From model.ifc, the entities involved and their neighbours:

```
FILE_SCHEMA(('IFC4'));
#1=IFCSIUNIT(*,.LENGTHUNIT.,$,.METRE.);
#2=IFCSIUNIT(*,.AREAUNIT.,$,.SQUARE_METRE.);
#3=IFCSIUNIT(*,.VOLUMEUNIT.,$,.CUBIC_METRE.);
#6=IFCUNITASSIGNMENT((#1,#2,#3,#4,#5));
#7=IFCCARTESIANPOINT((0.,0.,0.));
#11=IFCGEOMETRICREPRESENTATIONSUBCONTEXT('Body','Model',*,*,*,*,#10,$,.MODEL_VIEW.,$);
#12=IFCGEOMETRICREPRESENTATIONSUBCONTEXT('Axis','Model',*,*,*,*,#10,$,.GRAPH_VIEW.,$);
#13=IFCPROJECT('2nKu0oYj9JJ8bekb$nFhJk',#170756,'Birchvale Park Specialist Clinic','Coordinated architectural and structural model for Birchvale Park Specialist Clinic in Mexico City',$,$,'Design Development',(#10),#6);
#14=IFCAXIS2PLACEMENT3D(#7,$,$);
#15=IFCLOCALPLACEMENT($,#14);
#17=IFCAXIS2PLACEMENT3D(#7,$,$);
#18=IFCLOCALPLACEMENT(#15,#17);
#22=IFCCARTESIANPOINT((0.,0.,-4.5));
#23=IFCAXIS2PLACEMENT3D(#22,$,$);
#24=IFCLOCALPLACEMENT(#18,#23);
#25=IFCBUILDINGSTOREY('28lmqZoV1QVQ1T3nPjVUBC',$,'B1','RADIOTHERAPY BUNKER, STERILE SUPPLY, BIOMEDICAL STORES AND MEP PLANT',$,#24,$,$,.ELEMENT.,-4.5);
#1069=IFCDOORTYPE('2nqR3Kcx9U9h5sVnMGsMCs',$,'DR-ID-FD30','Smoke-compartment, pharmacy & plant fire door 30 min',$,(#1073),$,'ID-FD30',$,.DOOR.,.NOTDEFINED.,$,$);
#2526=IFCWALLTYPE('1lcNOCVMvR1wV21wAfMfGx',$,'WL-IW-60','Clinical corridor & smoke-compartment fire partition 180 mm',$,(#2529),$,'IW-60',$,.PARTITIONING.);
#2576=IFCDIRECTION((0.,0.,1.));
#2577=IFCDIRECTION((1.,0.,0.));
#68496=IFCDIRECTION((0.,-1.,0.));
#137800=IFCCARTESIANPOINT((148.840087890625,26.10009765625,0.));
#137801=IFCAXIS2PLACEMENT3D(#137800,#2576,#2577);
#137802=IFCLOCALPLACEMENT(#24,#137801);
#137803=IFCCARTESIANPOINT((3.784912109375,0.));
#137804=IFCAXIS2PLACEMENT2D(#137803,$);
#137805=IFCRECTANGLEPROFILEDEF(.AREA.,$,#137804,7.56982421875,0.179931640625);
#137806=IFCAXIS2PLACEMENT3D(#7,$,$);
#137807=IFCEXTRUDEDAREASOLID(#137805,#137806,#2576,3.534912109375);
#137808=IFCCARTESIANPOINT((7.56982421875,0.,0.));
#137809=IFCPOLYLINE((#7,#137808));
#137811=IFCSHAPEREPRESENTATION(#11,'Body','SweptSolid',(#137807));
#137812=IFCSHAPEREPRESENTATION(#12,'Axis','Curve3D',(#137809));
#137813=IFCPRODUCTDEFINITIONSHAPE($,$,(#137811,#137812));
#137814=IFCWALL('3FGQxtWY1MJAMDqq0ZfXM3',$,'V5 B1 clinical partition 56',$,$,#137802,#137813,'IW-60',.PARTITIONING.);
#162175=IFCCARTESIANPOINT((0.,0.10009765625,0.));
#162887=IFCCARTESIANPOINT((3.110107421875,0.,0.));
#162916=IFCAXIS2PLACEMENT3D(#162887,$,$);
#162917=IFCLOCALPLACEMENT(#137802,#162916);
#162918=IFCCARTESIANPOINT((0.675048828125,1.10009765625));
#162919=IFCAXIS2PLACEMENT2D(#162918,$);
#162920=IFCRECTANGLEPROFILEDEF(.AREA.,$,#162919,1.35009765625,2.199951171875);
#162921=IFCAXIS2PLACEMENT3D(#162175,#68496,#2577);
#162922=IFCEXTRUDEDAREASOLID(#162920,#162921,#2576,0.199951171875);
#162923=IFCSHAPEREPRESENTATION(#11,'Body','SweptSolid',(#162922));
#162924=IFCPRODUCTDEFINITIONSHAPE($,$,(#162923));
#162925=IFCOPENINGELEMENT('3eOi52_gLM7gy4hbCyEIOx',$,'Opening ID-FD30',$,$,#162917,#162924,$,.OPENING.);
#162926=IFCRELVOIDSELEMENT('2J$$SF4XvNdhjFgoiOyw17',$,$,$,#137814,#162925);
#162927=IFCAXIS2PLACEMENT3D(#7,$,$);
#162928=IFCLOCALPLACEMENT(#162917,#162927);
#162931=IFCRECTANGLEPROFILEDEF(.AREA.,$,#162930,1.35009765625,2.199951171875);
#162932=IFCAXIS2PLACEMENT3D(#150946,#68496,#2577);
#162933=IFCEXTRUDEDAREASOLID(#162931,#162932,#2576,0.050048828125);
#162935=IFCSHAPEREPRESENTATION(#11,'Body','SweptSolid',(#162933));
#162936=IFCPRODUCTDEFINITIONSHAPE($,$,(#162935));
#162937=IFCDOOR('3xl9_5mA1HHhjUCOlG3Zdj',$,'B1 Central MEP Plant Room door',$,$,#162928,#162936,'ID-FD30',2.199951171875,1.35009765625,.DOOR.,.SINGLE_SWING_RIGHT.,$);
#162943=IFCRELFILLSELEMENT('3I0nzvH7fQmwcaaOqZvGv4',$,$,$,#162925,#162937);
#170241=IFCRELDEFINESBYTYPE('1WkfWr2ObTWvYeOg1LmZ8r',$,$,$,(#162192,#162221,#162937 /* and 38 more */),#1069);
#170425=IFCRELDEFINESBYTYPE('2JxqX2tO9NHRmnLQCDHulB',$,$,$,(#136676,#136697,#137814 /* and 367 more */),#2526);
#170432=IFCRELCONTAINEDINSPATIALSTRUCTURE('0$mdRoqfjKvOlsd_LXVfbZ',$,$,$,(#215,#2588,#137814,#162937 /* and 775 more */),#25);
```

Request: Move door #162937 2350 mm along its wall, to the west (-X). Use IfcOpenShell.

```python
import ifcopenshell
import ifcopenshell.api.geometry
import ifcopenshell.util.placement
import ifcopenshell.util.unit

model = ifcopenshell.open("model.ifc")
unit_scale = ifcopenshell.util.unit.calculate_unit_scale(model)

door = model.by_guid("3xl9_5mA1HHhjUCOlG3Zdj")
opening = door.FillsVoids[0].RelatingOpeningElement
wall = opening.VoidsElements[0].RelatingBuildingElement

wall_matrix = ifcopenshell.util.placement.get_local_placement(wall.ObjectPlacement)
shift = wall_matrix[:3, 0] * -2.35 / unit_scale
before = ifcopenshell.util.placement.get_local_placement(door.ObjectPlacement)[:3, 3].copy()

# The door is placed relative to its opening, so it follows when the opening moves.
matrix = ifcopenshell.util.placement.get_local_placement(opening.ObjectPlacement)
matrix[:3, 3] += shift
ifcopenshell.api.geometry.edit_object_placement(
    model, product=opening, matrix=matrix, is_si=False, should_transform_children=True
)

after = ifcopenshell.util.placement.get_local_placement(door.ObjectPlacement)[:3, 3]
print("door moved by", (after - before).round(3) + 0.0)

model.write("model_v2.ifc")
```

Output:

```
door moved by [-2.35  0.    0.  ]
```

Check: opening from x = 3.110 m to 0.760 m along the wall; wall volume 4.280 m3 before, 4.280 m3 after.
